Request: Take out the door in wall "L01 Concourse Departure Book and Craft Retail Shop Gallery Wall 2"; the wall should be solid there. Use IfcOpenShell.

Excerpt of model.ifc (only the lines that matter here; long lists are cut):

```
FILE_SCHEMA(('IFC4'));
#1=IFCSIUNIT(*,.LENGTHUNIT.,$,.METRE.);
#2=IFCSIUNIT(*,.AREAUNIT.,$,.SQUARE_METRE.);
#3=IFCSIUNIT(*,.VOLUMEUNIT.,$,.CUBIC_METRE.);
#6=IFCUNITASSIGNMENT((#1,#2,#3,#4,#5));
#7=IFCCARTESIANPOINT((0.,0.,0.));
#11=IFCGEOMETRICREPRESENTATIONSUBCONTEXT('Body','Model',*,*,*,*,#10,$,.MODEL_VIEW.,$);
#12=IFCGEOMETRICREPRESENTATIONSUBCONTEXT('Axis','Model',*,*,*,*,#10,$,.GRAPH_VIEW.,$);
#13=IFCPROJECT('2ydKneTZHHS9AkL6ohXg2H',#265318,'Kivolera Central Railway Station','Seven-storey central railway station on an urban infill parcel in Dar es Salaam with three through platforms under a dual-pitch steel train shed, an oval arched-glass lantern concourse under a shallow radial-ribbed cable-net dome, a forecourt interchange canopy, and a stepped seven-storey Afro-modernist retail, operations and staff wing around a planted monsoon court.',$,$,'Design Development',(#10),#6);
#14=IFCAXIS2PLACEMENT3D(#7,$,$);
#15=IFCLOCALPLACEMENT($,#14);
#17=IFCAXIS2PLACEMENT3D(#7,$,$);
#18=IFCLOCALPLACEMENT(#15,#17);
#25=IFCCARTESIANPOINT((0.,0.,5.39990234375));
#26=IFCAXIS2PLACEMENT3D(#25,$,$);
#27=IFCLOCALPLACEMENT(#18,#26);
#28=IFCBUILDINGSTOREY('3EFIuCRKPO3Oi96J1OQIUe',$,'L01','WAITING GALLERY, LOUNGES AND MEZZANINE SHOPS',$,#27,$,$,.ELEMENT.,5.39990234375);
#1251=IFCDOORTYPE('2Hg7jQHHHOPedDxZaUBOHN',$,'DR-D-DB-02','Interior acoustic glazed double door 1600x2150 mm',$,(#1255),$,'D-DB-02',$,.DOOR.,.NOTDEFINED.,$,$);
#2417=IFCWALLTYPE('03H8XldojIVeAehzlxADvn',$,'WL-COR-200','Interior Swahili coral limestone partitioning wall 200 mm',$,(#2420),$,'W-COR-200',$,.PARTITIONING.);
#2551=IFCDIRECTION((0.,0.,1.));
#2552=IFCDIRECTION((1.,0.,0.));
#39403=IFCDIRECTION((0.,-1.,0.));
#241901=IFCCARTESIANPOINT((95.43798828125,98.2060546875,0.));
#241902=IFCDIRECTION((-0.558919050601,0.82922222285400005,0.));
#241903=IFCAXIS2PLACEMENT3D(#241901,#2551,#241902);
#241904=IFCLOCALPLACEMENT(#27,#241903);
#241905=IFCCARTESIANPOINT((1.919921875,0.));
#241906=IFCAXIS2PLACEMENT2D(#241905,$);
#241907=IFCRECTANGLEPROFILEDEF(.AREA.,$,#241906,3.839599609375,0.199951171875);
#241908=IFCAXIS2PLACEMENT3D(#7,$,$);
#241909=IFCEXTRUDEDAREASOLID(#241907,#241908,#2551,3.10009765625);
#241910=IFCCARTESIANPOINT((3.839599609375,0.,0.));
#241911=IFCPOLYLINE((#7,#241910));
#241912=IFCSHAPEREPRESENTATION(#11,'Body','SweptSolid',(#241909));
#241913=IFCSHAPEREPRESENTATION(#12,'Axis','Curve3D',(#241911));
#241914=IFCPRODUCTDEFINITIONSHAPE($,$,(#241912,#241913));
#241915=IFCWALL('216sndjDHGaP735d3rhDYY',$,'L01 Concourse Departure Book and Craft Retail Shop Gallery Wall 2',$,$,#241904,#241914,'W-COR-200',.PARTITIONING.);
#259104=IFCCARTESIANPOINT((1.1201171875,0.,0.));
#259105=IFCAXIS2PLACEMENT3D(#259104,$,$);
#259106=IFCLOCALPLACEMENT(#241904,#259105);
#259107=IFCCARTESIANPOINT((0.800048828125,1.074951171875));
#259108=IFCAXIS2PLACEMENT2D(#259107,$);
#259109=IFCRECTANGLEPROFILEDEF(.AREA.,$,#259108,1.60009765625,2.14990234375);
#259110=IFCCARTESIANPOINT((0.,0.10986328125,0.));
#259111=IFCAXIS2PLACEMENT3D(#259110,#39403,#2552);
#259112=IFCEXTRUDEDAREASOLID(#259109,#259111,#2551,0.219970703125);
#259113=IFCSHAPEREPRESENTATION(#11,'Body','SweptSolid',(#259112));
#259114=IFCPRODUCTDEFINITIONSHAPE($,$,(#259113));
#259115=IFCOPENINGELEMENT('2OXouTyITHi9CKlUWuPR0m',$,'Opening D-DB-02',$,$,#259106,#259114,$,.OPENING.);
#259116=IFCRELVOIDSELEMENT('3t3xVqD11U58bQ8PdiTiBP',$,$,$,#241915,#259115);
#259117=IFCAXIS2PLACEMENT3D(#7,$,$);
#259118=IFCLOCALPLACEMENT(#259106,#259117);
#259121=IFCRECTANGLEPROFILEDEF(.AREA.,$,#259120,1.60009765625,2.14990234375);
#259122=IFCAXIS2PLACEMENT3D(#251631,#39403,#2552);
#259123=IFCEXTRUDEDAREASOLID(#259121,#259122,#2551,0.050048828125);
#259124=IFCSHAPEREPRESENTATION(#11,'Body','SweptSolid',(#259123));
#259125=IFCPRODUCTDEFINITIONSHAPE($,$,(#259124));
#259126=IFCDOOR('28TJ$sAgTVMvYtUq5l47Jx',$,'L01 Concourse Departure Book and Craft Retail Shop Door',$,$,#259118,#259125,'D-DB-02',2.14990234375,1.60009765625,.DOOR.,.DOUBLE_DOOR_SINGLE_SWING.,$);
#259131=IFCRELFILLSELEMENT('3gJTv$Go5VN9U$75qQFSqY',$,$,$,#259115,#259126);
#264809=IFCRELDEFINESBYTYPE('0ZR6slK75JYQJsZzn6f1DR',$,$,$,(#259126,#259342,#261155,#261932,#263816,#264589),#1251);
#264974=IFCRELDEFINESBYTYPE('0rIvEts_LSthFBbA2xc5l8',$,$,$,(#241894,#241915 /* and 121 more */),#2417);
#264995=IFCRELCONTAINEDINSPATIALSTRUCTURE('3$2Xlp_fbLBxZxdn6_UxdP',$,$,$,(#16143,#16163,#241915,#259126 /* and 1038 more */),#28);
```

```python
import ifcopenshell
import ifcopenshell.api.feature
import ifcopenshell.api.root
import ifcopenshell.geom
import ifcopenshell.util.shape

model = ifcopenshell.open("model.ifc")
settings = ifcopenshell.geom.settings()


def volume(element):
    """Net volume in cubic metres, openings subtracted."""
    shape = ifcopenshell.geom.create_shape(settings, element)
    return ifcopenshell.util.shape.get_volume(shape.geometry)


door = model.by_id(259126)
opening = door.FillsVoids[0].RelatingOpeningElement
wall = opening.VoidsElements[0].RelatingBuildingElement
before = volume(wall)

ifcopenshell.api.root.remove_product(model, product=door)
ifcopenshell.api.feature.remove_feature(model, feature=opening)

after = volume(wall)

print(f"wall volume {before:.3f} -> {after:.3f} m3")

model.write("model_updated.ifc")
```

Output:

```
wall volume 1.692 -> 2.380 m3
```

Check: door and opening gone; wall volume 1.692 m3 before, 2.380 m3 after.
